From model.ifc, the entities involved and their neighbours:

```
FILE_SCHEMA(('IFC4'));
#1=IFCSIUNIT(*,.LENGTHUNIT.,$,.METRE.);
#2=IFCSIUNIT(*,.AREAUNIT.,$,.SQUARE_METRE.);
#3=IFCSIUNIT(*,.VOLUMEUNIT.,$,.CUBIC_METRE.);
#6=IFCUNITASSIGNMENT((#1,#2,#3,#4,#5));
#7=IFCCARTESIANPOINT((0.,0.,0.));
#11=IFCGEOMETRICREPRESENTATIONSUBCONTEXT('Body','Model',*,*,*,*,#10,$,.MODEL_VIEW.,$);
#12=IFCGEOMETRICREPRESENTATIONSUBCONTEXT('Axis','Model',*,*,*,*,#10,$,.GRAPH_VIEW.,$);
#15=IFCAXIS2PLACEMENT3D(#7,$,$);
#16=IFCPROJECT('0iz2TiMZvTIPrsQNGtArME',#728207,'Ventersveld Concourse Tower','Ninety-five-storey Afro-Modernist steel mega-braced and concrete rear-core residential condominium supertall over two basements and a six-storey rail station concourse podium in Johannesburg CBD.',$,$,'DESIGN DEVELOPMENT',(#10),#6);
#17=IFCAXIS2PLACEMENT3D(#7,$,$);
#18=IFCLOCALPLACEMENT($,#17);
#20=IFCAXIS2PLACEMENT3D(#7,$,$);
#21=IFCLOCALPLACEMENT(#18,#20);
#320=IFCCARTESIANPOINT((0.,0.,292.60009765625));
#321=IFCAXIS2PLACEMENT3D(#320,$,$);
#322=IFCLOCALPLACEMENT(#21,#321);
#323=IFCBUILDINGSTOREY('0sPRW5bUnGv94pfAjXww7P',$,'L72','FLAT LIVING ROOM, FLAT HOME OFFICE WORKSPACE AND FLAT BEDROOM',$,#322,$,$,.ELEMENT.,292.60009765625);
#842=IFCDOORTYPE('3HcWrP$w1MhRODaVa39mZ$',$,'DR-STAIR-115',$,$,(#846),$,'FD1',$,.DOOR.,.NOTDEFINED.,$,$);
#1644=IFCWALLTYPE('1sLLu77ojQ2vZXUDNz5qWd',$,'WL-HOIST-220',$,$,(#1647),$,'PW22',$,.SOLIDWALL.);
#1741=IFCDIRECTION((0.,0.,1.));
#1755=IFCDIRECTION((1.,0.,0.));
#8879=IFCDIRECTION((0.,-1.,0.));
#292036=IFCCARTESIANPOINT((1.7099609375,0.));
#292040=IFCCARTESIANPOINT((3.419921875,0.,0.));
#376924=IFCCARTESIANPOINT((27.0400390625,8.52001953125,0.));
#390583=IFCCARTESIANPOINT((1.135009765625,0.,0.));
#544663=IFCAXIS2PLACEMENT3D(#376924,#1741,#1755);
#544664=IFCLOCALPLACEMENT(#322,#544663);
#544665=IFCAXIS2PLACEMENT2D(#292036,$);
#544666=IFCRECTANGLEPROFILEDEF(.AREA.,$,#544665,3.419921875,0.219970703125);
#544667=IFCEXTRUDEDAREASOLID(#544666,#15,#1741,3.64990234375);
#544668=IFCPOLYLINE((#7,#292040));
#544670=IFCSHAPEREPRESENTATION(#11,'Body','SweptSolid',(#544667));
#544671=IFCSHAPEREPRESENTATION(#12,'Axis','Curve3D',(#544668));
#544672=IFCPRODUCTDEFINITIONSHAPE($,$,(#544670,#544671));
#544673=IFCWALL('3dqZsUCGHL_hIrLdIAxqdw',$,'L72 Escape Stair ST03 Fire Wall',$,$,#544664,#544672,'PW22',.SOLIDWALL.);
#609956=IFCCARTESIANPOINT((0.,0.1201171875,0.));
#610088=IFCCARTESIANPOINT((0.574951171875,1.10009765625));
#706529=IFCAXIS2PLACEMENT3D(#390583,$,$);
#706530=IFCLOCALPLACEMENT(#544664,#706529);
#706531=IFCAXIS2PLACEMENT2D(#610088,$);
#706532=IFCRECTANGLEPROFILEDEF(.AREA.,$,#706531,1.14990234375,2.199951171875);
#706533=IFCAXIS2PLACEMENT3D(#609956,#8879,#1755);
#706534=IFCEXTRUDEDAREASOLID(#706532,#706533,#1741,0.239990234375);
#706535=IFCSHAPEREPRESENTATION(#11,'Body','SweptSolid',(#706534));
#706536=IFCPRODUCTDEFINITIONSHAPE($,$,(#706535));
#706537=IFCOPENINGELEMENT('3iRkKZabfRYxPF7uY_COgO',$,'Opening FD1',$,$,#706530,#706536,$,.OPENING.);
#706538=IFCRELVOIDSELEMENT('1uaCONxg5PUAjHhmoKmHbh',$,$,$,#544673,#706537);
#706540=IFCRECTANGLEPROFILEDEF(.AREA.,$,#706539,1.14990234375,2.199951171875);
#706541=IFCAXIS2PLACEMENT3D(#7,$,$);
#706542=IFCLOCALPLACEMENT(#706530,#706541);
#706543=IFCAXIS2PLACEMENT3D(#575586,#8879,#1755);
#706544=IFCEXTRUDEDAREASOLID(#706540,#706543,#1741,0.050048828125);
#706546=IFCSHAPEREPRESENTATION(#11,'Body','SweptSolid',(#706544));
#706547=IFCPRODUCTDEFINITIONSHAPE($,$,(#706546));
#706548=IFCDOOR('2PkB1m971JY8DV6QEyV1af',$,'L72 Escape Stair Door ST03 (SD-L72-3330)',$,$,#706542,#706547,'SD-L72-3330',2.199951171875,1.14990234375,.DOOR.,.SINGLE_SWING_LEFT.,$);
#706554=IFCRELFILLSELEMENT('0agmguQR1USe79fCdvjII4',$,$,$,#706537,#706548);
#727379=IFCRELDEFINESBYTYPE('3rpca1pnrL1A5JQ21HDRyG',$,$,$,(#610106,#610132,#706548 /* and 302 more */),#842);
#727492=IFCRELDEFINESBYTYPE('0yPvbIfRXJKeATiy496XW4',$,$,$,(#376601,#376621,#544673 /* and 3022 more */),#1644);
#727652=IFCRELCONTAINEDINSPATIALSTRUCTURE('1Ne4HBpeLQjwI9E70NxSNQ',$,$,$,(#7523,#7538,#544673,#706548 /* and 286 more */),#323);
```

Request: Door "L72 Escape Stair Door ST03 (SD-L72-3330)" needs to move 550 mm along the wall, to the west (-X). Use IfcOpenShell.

```python
import ifcopenshell
import ifcopenshell.api.geometry
import ifcopenshell.util.placement
import ifcopenshell.util.unit

model = ifcopenshell.open("model.ifc")
unit_scale = ifcopenshell.util.unit.calculate_unit_scale(model)

door = model.by_guid("2PkB1m971JY8DV6QEyV1af")
opening = door.FillsVoids[0].RelatingOpeningElement
wall = opening.VoidsElements[0].RelatingBuildingElement

wall_matrix = ifcopenshell.util.placement.get_local_placement(wall.ObjectPlacement)
shift = wall_matrix[:3, 0] * -0.55 / unit_scale
before = ifcopenshell.util.placement.get_local_placement(door.ObjectPlacement)[:3, 3].copy()

# The door is placed relative to its opening, so it follows when the opening moves.
matrix = ifcopenshell.util.placement.get_local_placement(opening.ObjectPlacement)
matrix[:3, 3] += shift
ifcopenshell.api.geometry.edit_object_placement(
    model, product=opening, matrix=matrix, is_si=False, should_transform_children=True
)

after = ifcopenshell.util.placement.get_local_placement(door.ObjectPlacement)[:3, 3]
print("door moved by", (after - before).round(3) + 0.0)

model.write("model_v2.ifc")
```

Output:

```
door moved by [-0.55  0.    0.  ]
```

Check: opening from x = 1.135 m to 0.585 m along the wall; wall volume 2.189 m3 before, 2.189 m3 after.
